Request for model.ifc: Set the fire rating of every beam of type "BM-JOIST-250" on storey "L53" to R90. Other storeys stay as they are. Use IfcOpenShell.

First a look at what the model holds.

```python
import ifcopenshell
import ifcopenshell.util.element

model = ifcopenshell.open("model.ifc")
print(model.schema)
storey = next(s for s in model.by_type("IfcBuildingStorey") if s.Name == "L53")
beams = [e for e in ifcopenshell.util.element.get_decomposition(storey) if e.is_a("IfcBeam")]
seen = {}
for e in beams:
    element_type = ifcopenshell.util.element.get_type(e)
    key = (element_type.Name if element_type != e and element_type else None, ifcopenshell.util.element.get_pset(e, "Pset_BeamCommon", "FireRating"))
    seen[key] = seen.get(key, 0) + 1
for (name, value), count in sorted(seen.items(), key=str):
    print(count, "x", name, "|", value)
```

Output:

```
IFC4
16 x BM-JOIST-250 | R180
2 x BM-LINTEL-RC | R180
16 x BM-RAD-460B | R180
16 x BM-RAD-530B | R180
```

```python
import ifcopenshell
import ifcopenshell.api.pset
import ifcopenshell.util.element

model = ifcopenshell.open("model.ifc")

storey = next(s for s in model.by_type("IfcBuildingStorey") if s.Name == "L53")
beams = [e for e in ifcopenshell.util.element.get_decomposition(storey) if e.is_a("IfcBeam")]

count = 0
for e in beams:
    element_type = ifcopenshell.util.element.get_type(e)
    if element_type in (None, e) or element_type.Name != "BM-JOIST-250":
        continue
    found = ifcopenshell.util.element.get_pset(e, "Pset_BeamCommon", should_inherit=False)
    if found:
        pset = model.by_id(found["id"])
        if len(ifcopenshell.util.element.get_elements_by_pset(pset)) > 1:
            pset = ifcopenshell.api.pset.unshare_pset(model, products=[e], pset=pset)[0]
    else:
        pset = ifcopenshell.api.pset.add_pset(model, product=e, name="Pset_BeamCommon")
    ifcopenshell.api.pset.edit_pset(model, pset=pset, properties={"FireRating": "R90"})
    count += 1

print(count, "beams updated")

model.write("model_updated.ifc")
```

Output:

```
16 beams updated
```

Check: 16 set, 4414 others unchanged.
